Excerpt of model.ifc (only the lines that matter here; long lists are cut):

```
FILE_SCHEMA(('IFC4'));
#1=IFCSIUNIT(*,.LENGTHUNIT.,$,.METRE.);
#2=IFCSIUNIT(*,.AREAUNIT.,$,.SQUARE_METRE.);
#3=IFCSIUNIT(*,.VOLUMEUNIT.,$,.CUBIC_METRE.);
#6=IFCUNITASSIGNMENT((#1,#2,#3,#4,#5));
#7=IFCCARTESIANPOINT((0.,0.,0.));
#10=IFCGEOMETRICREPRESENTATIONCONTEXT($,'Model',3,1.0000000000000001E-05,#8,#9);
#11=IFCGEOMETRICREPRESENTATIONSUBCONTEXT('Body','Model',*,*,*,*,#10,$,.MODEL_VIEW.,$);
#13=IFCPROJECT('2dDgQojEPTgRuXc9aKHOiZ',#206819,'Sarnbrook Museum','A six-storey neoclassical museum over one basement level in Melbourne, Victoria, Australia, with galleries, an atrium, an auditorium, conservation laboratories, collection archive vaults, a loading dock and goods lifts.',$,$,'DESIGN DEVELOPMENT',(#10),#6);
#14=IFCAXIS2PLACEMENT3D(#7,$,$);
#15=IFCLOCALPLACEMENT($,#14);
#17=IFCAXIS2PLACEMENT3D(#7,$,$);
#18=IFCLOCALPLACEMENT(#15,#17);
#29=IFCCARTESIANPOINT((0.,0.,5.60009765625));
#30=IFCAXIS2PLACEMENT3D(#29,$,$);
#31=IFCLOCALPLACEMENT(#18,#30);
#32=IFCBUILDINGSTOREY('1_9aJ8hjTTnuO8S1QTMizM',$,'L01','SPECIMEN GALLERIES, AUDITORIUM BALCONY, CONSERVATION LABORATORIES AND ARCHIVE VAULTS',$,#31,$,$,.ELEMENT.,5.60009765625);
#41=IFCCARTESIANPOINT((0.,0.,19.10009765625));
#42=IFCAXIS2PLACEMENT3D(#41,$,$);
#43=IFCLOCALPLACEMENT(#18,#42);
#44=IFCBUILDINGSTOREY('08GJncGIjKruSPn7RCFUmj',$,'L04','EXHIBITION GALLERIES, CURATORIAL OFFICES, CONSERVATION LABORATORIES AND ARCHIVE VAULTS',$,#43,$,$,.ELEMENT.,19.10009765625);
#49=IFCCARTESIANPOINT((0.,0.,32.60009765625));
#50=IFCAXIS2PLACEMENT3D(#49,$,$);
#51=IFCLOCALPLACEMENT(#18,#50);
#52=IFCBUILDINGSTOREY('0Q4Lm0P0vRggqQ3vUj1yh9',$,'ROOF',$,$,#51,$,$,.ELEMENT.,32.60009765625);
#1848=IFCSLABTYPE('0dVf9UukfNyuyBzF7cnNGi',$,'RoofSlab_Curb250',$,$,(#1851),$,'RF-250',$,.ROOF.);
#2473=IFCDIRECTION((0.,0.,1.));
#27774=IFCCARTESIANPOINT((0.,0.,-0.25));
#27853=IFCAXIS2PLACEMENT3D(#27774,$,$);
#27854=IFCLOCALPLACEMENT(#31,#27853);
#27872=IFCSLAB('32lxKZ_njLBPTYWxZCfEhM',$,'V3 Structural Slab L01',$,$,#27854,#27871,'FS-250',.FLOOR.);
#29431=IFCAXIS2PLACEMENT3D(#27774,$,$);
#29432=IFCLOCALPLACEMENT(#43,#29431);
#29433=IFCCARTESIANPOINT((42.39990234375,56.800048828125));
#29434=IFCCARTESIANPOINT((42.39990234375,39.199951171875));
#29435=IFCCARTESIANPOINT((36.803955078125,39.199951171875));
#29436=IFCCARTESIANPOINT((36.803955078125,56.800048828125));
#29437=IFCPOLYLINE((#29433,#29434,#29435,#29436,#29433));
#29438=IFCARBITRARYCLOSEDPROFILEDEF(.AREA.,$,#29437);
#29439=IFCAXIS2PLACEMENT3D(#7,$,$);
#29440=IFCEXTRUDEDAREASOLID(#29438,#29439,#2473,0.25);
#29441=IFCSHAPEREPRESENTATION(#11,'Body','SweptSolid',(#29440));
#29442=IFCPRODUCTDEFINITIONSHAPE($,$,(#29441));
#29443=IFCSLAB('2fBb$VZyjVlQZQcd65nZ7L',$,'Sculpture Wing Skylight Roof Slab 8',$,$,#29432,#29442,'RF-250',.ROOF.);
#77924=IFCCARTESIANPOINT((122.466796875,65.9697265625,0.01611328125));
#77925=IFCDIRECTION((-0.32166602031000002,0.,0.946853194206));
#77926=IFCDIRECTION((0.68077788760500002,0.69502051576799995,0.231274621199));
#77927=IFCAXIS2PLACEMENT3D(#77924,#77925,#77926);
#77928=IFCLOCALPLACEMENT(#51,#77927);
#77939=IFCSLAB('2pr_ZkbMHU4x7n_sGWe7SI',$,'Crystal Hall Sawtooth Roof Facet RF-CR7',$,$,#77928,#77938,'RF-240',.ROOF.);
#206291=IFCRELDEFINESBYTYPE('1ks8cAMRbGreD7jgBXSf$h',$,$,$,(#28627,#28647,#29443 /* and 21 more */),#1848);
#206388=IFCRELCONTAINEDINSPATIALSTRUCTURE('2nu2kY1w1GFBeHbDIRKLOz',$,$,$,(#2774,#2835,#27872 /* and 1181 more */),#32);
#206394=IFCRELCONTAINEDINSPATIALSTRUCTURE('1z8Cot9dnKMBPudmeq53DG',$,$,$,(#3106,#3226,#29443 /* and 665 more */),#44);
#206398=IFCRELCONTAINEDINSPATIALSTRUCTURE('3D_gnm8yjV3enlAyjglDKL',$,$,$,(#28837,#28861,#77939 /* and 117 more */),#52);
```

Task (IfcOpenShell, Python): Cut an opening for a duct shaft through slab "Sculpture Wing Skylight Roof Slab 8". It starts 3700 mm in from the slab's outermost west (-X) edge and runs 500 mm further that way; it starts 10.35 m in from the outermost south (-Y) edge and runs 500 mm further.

```python
import numpy as np
import ifcopenshell
import ifcopenshell.api.feature
import ifcopenshell.api.geometry
import ifcopenshell.api.root
import ifcopenshell.geom
import ifcopenshell.util.placement
import ifcopenshell.util.representation
import ifcopenshell.util.shape
import ifcopenshell.util.unit

model = ifcopenshell.open("model.ifc")
unit_scale = ifcopenshell.util.unit.calculate_unit_scale(model)
settings = ifcopenshell.geom.settings()


def volume(element):
    """Net volume in cubic metres, openings subtracted."""
    shape = ifcopenshell.geom.create_shape(settings, element)
    return ifcopenshell.util.shape.get_volume(shape.geometry)


slab = model.by_id(29443)
before = volume(slab)

# Extent in the slab's own axes, in metres. The edges named are its -X and -Y sides.
slab_shape = ifcopenshell.geom.create_shape(settings, slab)
vertices = ifcopenshell.util.shape.get_vertices(slab_shape.geometry)
x_min, y_min, bottom = vertices.min(axis=0)
top = vertices[:, 2].max()

opening = ifcopenshell.api.root.create_entity(model, ifc_class="IfcOpeningElement", name="Duct shaft opening", predefined_type="OPENING")
context = ifcopenshell.util.representation.get_context(model, "Model", "Body", "MODEL_VIEW")
width, depth = 0.5, 0.5
outline = [(0.0, 0.0), (width, 0.0), (width, depth), (0.0, depth), (0.0, 0.0)]
# Overshoot both faces by 50 mm so the cut is clean.
shape = ifcopenshell.api.geometry.add_slab_representation(
    model, context=context, depth=top - bottom + 0.1, polyline=outline
)
ifcopenshell.api.geometry.assign_representation(model, product=opening, representation=shape)

matrix = ifcopenshell.util.placement.get_local_placement(slab.ObjectPlacement)
matrix[:, 3] = matrix @ np.append(np.array([x_min + 3.7, y_min + 10.35, bottom - 0.05]) / unit_scale, 1.0)
ifcopenshell.api.geometry.edit_object_placement(model, product=opening, matrix=matrix, is_si=False)
ifcopenshell.api.feature.add_feature(model, feature=opening, element=slab)

after = volume(slab)

print(f"slab volume {before:.3f} -> {after:.3f} m3")

model.write("model_rev.ifc")
```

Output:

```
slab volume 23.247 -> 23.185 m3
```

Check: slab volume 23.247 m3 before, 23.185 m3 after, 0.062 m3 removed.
